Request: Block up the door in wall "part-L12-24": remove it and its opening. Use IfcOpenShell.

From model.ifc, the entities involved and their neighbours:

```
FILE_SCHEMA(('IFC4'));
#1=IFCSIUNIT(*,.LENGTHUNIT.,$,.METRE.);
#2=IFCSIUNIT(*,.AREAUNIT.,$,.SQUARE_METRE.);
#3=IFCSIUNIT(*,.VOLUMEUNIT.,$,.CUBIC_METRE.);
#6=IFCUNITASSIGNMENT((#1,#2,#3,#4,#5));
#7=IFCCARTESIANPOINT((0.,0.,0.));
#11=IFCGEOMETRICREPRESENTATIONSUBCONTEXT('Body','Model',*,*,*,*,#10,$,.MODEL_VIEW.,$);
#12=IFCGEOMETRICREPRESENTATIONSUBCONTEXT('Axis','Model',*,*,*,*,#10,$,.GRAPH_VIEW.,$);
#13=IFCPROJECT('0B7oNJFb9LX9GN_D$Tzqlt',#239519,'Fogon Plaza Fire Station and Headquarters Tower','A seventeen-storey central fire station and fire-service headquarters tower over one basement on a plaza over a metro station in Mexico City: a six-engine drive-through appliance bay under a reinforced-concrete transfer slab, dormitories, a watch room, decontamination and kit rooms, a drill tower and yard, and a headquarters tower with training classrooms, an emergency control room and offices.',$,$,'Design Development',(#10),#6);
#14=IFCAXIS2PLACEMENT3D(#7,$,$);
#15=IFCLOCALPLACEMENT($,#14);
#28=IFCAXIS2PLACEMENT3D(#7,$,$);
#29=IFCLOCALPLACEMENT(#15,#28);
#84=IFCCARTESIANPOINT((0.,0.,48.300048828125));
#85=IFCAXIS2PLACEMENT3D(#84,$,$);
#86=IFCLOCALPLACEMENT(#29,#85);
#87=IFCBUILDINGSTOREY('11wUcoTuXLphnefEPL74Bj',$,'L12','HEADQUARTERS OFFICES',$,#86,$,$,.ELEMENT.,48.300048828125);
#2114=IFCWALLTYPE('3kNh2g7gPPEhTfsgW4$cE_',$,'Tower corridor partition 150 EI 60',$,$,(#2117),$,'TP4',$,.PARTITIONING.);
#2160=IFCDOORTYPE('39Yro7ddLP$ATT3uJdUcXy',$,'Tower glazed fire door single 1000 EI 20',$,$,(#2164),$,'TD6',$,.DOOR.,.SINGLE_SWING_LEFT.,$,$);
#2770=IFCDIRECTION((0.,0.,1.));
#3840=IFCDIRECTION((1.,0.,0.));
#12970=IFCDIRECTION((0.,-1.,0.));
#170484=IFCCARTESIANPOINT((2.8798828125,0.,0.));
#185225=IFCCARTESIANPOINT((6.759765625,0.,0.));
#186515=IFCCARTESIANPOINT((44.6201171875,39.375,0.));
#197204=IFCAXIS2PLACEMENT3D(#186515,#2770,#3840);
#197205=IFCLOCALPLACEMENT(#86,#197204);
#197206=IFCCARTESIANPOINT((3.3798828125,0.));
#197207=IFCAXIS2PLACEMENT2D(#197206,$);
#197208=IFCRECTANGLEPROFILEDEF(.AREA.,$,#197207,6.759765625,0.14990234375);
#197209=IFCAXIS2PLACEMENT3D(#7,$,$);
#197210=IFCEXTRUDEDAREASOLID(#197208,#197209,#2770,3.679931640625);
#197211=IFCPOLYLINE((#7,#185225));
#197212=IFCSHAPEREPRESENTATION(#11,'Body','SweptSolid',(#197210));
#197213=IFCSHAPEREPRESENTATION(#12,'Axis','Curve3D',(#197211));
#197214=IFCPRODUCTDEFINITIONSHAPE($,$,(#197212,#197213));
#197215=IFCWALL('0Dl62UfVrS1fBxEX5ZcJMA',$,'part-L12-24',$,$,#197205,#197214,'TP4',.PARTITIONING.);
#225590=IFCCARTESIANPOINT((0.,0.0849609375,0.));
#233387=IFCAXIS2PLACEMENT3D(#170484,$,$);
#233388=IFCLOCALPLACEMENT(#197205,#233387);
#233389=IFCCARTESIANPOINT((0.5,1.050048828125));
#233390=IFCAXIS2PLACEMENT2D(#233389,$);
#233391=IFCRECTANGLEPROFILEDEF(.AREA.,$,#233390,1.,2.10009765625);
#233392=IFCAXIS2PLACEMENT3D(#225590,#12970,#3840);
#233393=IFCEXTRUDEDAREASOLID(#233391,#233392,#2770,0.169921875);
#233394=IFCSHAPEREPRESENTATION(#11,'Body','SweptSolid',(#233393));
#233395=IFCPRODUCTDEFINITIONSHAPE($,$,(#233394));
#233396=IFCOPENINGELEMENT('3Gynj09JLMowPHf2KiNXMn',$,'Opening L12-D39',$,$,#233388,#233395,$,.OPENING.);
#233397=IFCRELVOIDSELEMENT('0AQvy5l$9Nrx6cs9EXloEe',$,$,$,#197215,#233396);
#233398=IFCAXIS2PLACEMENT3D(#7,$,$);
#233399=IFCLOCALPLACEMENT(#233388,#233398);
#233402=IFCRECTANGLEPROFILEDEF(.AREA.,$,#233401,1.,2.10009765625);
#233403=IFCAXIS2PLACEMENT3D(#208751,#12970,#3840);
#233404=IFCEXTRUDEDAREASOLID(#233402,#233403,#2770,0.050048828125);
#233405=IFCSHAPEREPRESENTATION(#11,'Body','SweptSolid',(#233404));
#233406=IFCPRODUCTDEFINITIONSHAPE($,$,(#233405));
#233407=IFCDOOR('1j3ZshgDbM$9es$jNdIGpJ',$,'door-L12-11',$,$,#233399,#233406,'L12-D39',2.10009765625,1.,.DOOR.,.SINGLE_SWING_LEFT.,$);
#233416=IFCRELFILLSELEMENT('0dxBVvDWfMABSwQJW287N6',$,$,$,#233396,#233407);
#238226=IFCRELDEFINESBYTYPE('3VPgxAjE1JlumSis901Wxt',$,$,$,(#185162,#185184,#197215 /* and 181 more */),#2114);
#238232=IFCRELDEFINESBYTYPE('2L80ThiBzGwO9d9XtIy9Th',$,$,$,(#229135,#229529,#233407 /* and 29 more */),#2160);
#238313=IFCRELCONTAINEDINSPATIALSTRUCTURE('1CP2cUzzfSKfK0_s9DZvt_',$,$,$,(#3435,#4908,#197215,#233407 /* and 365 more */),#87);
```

```python
import ifcopenshell
import ifcopenshell.api.feature
import ifcopenshell.api.root
import ifcopenshell.geom
import ifcopenshell.util.shape

model = ifcopenshell.open("model.ifc")
settings = ifcopenshell.geom.settings()


def volume(element):
    """Net volume in cubic metres, openings subtracted."""
    shape = ifcopenshell.geom.create_shape(settings, element)
    return ifcopenshell.util.shape.get_volume(shape.geometry)


door = model.by_guid("1j3ZshgDbM$9es$jNdIGpJ")
opening = door.FillsVoids[0].RelatingOpeningElement
wall = opening.VoidsElements[0].RelatingBuildingElement
before = volume(wall)

ifcopenshell.api.root.remove_product(model, product=door)
ifcopenshell.api.feature.remove_feature(model, feature=opening)

after = volume(wall)

print(f"wall volume {before:.3f} -> {after:.3f} m3")

model.write("model-out.ifc")
```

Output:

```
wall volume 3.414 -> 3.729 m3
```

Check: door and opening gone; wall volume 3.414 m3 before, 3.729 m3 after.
